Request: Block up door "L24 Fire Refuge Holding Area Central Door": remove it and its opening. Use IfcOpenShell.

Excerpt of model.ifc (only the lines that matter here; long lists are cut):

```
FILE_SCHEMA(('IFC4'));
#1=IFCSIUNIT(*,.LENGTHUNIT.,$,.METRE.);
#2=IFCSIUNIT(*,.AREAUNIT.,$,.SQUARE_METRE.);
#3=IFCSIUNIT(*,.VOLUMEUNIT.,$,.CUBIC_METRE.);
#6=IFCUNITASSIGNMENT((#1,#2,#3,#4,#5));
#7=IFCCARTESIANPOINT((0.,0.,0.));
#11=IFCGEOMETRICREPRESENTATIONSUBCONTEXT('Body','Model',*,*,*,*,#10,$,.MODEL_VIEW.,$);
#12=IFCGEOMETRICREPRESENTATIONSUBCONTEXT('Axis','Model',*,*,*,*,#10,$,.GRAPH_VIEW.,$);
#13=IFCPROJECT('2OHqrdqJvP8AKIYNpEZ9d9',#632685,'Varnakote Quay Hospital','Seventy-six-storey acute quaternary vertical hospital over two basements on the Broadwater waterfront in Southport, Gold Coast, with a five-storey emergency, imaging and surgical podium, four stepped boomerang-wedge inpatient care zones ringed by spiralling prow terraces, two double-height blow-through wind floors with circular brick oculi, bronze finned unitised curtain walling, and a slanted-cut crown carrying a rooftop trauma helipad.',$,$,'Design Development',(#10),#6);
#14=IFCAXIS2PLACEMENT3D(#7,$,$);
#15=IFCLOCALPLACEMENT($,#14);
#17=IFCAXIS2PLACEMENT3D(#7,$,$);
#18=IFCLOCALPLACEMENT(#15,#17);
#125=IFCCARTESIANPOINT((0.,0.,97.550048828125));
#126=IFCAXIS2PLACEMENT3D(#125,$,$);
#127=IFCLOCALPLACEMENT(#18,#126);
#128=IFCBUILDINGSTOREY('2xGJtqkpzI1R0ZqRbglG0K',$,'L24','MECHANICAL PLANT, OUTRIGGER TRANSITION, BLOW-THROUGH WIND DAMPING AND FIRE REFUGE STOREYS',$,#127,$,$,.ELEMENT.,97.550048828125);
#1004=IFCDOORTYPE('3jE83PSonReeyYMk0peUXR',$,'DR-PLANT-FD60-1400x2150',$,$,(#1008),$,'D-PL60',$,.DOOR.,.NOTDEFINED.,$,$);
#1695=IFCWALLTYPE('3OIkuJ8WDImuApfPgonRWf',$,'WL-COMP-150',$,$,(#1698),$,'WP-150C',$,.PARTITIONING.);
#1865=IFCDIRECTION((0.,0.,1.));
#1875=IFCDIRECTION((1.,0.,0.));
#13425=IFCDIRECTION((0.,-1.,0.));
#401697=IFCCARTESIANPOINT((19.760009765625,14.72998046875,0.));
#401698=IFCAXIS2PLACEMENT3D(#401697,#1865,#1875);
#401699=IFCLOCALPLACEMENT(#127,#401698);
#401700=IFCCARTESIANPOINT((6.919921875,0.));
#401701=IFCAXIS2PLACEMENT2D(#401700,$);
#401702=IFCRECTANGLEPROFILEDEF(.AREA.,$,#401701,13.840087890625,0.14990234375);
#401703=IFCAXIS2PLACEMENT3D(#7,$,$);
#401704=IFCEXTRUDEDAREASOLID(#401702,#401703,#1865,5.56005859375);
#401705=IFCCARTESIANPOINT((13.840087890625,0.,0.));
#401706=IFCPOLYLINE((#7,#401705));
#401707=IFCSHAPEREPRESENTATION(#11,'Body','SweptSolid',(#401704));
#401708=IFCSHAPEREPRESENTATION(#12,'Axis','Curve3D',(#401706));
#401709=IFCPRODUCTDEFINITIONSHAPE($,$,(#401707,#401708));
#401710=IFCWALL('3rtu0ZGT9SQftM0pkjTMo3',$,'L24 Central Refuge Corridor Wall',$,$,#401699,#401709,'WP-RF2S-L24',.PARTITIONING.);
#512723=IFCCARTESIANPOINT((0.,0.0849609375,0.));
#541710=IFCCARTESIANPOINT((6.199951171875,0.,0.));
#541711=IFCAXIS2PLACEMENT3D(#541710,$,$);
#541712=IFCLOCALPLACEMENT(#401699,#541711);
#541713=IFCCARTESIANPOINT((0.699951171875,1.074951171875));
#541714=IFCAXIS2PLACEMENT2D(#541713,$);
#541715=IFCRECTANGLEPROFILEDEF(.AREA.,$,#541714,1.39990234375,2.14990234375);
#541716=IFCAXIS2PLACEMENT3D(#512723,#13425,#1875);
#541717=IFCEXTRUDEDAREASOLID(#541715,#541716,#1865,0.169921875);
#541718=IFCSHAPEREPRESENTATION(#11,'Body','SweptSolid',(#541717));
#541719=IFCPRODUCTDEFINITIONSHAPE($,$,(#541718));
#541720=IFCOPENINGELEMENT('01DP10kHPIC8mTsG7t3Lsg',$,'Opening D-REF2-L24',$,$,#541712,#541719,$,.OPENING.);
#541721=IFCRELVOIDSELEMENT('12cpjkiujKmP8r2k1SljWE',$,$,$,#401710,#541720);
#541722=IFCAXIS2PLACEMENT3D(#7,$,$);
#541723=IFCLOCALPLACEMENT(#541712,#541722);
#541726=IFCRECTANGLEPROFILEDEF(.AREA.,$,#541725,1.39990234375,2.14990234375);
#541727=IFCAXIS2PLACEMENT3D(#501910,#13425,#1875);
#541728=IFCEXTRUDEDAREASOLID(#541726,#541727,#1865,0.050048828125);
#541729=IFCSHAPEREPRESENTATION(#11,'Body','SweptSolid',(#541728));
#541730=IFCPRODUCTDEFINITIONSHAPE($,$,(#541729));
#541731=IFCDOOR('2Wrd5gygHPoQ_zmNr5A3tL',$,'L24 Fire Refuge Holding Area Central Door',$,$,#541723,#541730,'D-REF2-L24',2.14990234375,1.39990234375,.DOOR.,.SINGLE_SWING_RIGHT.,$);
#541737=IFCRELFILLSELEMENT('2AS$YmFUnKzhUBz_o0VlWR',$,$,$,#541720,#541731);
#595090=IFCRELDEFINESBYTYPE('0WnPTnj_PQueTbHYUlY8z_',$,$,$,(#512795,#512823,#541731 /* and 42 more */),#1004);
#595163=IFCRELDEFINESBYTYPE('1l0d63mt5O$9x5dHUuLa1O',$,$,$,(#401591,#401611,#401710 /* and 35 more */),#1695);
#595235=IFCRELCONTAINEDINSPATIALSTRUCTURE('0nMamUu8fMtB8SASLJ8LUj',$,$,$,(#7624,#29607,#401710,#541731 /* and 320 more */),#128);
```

```python
import ifcopenshell
import ifcopenshell.api.feature
import ifcopenshell.api.root
import ifcopenshell.geom
import ifcopenshell.util.shape

model = ifcopenshell.open("model.ifc")
settings = ifcopenshell.geom.settings()


def volume(element):
    """Net volume in cubic metres, openings subtracted."""
    shape = ifcopenshell.geom.create_shape(settings, element)
    return ifcopenshell.util.shape.get_volume(shape.geometry)


door = model.by_guid("2Wrd5gygHPoQ_zmNr5A3tL")
opening = door.FillsVoids[0].RelatingOpeningElement
wall = opening.VoidsElements[0].RelatingBuildingElement
before = volume(wall)

ifcopenshell.api.root.remove_product(model, product=door)
ifcopenshell.api.feature.remove_feature(model, feature=opening)

after = volume(wall)

print(f"wall volume {before:.3f} -> {after:.3f} m3")

model.write("model_v2.ifc")
```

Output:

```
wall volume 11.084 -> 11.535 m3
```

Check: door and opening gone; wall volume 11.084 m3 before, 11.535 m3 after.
